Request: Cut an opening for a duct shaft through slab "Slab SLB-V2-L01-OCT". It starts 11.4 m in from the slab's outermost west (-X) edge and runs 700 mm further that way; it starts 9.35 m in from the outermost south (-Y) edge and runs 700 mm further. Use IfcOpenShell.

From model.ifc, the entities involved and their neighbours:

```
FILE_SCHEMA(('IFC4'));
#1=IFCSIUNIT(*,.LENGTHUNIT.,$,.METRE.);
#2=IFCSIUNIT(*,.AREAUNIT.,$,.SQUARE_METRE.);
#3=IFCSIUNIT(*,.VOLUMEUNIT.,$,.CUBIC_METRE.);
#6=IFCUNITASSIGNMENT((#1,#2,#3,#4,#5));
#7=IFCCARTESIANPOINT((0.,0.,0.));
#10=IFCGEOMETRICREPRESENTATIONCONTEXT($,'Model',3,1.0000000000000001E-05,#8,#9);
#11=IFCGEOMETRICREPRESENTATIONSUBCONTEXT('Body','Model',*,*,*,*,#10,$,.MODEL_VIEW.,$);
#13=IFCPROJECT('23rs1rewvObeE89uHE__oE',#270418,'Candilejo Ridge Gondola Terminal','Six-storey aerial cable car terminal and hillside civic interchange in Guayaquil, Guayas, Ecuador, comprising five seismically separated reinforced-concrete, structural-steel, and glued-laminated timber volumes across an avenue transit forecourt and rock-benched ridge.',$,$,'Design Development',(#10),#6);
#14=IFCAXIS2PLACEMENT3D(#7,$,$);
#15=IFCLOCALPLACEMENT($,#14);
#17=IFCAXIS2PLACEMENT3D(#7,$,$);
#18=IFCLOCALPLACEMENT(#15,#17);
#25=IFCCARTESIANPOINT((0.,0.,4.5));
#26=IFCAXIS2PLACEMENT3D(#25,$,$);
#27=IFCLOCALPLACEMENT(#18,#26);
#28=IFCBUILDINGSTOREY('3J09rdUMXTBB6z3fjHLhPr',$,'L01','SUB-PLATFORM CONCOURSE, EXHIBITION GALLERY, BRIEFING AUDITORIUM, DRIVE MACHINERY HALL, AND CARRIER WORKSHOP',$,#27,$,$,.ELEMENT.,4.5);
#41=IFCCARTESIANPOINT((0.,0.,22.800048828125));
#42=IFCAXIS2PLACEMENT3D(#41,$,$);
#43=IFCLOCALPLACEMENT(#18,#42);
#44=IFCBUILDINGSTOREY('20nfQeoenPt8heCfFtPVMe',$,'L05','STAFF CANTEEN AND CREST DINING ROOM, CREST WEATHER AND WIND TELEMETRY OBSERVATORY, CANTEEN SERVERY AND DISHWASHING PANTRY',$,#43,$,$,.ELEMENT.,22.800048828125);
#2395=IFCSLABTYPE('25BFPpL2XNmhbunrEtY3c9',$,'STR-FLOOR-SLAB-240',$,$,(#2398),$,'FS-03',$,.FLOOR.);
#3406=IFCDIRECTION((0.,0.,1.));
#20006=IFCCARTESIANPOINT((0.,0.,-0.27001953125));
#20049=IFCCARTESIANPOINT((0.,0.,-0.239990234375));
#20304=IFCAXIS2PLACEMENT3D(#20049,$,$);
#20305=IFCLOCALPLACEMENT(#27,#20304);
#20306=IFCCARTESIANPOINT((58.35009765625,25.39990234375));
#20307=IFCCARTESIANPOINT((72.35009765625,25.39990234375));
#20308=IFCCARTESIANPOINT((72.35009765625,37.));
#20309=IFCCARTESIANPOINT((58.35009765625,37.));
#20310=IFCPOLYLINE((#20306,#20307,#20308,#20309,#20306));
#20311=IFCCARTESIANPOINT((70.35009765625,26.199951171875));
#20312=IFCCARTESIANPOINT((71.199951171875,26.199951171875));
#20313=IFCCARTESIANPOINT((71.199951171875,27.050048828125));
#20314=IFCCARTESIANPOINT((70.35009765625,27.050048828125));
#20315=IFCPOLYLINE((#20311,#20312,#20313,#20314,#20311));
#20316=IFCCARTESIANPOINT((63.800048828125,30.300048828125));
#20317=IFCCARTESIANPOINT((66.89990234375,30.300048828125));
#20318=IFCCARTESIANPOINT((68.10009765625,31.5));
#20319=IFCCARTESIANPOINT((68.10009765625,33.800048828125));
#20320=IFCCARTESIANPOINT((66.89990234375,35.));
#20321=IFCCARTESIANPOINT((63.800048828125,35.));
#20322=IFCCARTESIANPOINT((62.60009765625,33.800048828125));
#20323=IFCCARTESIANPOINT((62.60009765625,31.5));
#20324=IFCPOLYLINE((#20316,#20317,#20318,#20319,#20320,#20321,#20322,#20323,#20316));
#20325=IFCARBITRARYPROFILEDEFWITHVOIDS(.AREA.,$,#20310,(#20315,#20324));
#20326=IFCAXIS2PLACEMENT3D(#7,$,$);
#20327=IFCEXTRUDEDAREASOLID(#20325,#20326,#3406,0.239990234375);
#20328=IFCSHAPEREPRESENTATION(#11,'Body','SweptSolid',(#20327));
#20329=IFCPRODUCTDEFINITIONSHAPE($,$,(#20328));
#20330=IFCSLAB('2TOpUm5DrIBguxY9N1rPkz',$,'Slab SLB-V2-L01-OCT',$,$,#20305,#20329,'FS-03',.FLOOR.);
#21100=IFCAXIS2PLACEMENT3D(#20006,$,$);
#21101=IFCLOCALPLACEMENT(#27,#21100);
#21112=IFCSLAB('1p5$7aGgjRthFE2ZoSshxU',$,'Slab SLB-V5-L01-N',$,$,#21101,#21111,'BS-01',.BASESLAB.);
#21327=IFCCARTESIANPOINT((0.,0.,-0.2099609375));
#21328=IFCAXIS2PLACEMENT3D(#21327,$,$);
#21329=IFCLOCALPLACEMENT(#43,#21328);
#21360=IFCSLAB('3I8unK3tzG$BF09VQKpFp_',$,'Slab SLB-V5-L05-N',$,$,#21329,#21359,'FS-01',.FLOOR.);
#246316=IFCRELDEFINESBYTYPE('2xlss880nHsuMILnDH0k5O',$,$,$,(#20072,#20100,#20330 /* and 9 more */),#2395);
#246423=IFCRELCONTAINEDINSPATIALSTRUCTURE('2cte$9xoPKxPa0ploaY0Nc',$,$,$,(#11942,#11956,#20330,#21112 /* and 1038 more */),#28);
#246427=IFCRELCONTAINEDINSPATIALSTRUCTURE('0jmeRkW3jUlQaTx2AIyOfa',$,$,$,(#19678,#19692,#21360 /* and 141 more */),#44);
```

```python
import numpy as np
import ifcopenshell
import ifcopenshell.api.feature
import ifcopenshell.api.geometry
import ifcopenshell.api.root
import ifcopenshell.geom
import ifcopenshell.util.placement
import ifcopenshell.util.representation
import ifcopenshell.util.shape
import ifcopenshell.util.unit

model = ifcopenshell.open("model.ifc")
unit_scale = ifcopenshell.util.unit.calculate_unit_scale(model)
settings = ifcopenshell.geom.settings()


def volume(element):
    """Net volume in cubic metres, openings subtracted."""
    shape = ifcopenshell.geom.create_shape(settings, element)
    return ifcopenshell.util.shape.get_volume(shape.geometry)


slab = model.by_guid("2TOpUm5DrIBguxY9N1rPkz")
before = volume(slab)

# Extent in the slab's own axes, in metres. The edges named are its -X and -Y sides.
slab_shape = ifcopenshell.geom.create_shape(settings, slab)
vertices = ifcopenshell.util.shape.get_vertices(slab_shape.geometry)
x_min, y_min, bottom = vertices.min(axis=0)
top = vertices[:, 2].max()

opening = ifcopenshell.api.root.create_entity(model, ifc_class="IfcOpeningElement", name="Duct shaft opening", predefined_type="OPENING")
context = ifcopenshell.util.representation.get_context(model, "Model", "Body", "MODEL_VIEW")
width, depth = 0.7, 0.7
outline = [(0.0, 0.0), (width, 0.0), (width, depth), (0.0, depth), (0.0, 0.0)]
# Overshoot both faces by 50 mm so the cut is clean.
shape = ifcopenshell.api.geometry.add_slab_representation(
    model, context=context, depth=top - bottom + 0.1, polyline=outline
)
ifcopenshell.api.geometry.assign_representation(model, product=opening, representation=shape)

matrix = ifcopenshell.util.placement.get_local_placement(slab.ObjectPlacement)
matrix[:, 3] = matrix @ np.append(np.array([x_min + 11.4, y_min + 9.35, bottom - 0.05]) / unit_scale, 1.0)
ifcopenshell.api.geometry.edit_object_placement(model, product=opening, matrix=matrix, is_si=False)
ifcopenshell.api.feature.add_feature(model, feature=opening, element=slab)

after = volume(slab)

print(f"slab volume {before:.3f} -> {after:.3f} m3")

model.write("model_rev.ifc")
```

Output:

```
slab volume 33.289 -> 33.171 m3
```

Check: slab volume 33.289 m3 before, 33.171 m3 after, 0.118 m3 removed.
